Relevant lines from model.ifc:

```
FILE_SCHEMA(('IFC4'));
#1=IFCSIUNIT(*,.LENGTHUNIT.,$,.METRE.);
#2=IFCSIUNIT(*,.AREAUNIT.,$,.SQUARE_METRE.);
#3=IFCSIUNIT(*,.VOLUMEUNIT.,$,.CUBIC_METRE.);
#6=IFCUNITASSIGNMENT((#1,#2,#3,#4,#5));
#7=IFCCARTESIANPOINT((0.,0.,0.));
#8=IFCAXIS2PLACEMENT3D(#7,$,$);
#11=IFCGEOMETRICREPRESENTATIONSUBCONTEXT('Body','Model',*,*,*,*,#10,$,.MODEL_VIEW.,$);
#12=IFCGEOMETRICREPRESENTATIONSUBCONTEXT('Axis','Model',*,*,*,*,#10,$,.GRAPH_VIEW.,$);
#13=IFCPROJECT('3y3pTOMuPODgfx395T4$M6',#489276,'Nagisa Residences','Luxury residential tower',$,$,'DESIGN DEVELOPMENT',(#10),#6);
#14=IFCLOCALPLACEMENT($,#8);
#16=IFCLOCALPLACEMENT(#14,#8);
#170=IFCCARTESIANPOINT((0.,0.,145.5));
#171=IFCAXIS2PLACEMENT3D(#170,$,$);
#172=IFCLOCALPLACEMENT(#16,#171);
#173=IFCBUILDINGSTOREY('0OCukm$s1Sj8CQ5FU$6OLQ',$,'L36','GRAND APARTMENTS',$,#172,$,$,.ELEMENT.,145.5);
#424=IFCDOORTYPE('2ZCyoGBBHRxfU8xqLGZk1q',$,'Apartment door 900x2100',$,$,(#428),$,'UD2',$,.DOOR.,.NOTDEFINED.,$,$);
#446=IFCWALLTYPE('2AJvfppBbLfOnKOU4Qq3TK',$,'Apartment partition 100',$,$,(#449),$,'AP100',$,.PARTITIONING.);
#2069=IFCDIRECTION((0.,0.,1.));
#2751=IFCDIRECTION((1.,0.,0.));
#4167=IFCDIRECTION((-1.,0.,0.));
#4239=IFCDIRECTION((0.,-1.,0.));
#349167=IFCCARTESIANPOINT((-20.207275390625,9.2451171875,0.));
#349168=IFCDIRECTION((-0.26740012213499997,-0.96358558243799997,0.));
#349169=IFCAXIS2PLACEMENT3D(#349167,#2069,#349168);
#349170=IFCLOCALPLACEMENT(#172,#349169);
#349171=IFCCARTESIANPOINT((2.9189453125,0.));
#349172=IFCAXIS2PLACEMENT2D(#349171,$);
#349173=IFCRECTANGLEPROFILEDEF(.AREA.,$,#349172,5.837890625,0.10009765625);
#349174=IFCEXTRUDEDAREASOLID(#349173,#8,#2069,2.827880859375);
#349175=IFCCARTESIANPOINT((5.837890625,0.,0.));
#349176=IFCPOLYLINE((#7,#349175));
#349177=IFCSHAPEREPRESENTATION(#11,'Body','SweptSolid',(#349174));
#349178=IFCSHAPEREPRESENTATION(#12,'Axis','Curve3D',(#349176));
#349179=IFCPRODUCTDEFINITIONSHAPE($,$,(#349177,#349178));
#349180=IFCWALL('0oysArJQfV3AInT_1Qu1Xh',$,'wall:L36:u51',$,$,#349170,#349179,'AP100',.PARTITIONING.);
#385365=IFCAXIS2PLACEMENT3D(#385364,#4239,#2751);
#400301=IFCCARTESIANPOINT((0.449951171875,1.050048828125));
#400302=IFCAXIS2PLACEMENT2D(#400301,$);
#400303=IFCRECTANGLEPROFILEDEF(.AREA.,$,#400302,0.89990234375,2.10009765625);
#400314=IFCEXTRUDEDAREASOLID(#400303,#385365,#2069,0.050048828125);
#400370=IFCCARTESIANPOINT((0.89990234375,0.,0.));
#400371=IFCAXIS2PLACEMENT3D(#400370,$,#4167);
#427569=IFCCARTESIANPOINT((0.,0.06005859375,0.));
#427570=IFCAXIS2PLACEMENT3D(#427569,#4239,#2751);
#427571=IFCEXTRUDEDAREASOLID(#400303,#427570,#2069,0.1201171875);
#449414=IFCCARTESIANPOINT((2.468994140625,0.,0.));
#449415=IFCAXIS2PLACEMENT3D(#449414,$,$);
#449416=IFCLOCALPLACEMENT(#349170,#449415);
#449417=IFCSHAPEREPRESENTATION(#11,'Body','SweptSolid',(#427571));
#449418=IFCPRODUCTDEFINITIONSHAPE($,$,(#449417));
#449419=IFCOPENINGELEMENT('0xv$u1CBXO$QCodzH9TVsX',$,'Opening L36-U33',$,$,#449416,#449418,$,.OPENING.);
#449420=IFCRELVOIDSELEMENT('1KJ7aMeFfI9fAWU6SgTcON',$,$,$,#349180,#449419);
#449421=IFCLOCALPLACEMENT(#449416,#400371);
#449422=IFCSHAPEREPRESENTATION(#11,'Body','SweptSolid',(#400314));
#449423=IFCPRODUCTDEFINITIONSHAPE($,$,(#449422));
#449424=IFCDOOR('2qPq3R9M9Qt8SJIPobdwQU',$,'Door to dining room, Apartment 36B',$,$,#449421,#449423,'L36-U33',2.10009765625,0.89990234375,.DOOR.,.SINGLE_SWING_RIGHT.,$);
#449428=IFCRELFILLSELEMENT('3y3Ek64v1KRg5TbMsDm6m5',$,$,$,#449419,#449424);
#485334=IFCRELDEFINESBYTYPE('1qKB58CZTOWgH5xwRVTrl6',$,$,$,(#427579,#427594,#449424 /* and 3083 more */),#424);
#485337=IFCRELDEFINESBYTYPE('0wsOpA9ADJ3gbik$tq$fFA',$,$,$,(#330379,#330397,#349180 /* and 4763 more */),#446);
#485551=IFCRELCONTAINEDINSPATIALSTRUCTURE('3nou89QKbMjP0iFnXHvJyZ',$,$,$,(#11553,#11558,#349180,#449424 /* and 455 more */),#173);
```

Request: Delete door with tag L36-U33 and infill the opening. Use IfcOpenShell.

```python
import ifcopenshell
import ifcopenshell.api.feature
import ifcopenshell.api.root
import ifcopenshell.geom
import ifcopenshell.util.shape

model = ifcopenshell.open("model.ifc")
settings = ifcopenshell.geom.settings()


def volume(element):
    """Net volume in cubic metres, openings subtracted."""
    shape = ifcopenshell.geom.create_shape(settings, element)
    return ifcopenshell.util.shape.get_volume(shape.geometry)


door = model.by_guid("2qPq3R9M9Qt8SJIPobdwQU")
opening = door.FillsVoids[0].RelatingOpeningElement
wall = opening.VoidsElements[0].RelatingBuildingElement
before = volume(wall)

ifcopenshell.api.root.remove_product(model, product=door)
ifcopenshell.api.feature.remove_feature(model, feature=opening)

after = volume(wall)

print(f"wall volume {before:.3f} -> {after:.3f} m3")

model.write("model_v2.ifc")
```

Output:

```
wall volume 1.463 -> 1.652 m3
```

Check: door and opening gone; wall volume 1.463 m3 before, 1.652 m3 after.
